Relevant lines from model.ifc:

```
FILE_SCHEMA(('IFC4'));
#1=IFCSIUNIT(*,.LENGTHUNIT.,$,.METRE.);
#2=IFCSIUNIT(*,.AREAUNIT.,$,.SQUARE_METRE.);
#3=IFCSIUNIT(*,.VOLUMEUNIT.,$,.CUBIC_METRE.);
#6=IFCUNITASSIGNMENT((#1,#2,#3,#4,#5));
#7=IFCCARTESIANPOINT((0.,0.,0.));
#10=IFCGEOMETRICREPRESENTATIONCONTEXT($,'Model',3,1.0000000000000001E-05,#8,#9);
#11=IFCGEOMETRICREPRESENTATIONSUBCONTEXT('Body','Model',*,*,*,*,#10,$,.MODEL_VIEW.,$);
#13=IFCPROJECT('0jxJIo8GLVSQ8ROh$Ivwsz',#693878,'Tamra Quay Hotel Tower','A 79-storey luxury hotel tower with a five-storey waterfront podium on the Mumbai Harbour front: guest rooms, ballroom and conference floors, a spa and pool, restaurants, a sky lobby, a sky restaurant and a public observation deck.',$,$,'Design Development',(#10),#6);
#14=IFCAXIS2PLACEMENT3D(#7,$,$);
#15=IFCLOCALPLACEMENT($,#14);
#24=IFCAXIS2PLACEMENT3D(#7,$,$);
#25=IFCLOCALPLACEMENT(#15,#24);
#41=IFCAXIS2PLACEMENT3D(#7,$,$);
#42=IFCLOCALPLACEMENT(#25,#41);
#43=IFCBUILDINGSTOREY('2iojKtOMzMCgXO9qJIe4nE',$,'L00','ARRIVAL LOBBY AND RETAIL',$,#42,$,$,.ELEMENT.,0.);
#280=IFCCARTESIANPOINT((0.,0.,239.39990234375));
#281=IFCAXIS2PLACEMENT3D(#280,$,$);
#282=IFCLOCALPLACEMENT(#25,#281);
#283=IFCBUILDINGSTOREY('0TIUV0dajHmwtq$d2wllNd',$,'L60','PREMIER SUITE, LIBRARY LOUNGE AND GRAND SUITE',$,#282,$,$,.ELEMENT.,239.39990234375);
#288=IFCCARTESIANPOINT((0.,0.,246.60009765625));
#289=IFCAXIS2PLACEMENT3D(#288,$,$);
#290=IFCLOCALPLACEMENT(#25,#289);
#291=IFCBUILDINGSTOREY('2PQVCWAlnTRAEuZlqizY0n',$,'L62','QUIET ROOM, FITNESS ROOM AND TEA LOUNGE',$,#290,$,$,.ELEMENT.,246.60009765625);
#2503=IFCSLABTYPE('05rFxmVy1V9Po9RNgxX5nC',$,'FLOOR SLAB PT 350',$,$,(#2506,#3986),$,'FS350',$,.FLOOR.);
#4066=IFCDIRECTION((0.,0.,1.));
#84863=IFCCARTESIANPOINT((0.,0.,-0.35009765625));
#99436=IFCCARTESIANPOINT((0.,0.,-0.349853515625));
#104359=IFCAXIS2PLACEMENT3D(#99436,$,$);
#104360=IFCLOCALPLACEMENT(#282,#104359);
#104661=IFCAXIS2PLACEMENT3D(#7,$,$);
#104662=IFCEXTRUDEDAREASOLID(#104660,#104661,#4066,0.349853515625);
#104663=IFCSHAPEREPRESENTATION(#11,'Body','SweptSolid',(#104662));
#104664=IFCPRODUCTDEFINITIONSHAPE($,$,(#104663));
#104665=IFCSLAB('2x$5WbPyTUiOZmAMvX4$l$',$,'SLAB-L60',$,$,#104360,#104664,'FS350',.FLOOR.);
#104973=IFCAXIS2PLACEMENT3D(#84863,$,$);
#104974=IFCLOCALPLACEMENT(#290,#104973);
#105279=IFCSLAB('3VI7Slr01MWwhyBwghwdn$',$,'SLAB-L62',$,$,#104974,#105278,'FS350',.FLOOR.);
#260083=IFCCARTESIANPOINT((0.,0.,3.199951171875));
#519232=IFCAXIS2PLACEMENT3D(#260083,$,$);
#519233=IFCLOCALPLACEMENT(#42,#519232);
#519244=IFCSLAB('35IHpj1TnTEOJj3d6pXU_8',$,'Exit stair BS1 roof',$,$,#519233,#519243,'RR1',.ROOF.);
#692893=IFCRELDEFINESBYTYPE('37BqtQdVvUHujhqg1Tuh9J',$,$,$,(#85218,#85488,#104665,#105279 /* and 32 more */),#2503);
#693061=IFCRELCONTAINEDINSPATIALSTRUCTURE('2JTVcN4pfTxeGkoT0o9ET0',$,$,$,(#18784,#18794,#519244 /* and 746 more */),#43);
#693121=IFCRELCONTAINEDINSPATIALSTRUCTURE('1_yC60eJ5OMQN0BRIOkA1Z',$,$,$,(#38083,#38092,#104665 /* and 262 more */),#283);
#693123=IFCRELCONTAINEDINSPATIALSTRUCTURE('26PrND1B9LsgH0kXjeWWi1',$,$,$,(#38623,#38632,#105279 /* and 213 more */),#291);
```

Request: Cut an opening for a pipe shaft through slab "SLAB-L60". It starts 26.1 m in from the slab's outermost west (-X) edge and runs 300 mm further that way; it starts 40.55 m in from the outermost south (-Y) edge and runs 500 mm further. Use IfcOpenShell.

```python
import numpy as np
import ifcopenshell
import ifcopenshell.api.feature
import ifcopenshell.api.geometry
import ifcopenshell.api.root
import ifcopenshell.geom
import ifcopenshell.util.placement
import ifcopenshell.util.representation
import ifcopenshell.util.shape
import ifcopenshell.util.unit

model = ifcopenshell.open("model.ifc")
unit_scale = ifcopenshell.util.unit.calculate_unit_scale(model)
settings = ifcopenshell.geom.settings()


def volume(element):
    """Net volume in cubic metres, openings subtracted."""
    shape = ifcopenshell.geom.create_shape(settings, element)
    return ifcopenshell.util.shape.get_volume(shape.geometry)


slab = model.by_guid("2x$5WbPyTUiOZmAMvX4$l$")
before = volume(slab)

# Extent in the slab's own axes, in metres. The edges named are its -X and -Y sides.
slab_shape = ifcopenshell.geom.create_shape(settings, slab)
vertices = ifcopenshell.util.shape.get_vertices(slab_shape.geometry)
x_min, y_min, bottom = vertices.min(axis=0)
top = vertices[:, 2].max()

opening = ifcopenshell.api.root.create_entity(model, ifc_class="IfcOpeningElement", name="Pipe shaft opening", predefined_type="OPENING")
context = ifcopenshell.util.representation.get_context(model, "Model", "Body", "MODEL_VIEW")
width, depth = 0.3, 0.5
outline = [(0.0, 0.0), (width, 0.0), (width, depth), (0.0, depth), (0.0, 0.0)]
# Overshoot both faces by 50 mm so the cut is clean.
shape = ifcopenshell.api.geometry.add_slab_representation(
    model, context=context, depth=top - bottom + 0.1, polyline=outline
)
ifcopenshell.api.geometry.assign_representation(model, product=opening, representation=shape)

matrix = ifcopenshell.util.placement.get_local_placement(slab.ObjectPlacement)
matrix[:, 3] = matrix @ np.append(np.array([x_min + 26.1, y_min + 40.55, bottom - 0.05]) / unit_scale, 1.0)
ifcopenshell.api.geometry.edit_object_placement(model, product=opening, matrix=matrix, is_si=False)
ifcopenshell.api.feature.add_feature(model, feature=opening, element=slab)

after = volume(slab)

print(f"slab volume {before:.3f} -> {after:.3f} m3")

model.write("model_edited.ifc")
```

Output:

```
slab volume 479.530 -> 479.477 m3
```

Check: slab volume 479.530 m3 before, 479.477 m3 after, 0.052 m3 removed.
